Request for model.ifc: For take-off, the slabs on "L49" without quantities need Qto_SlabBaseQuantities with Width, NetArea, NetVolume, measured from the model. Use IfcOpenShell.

First a look at what the model holds.

```python
import ifcopenshell
import ifcopenshell.util.element
import ifcopenshell.util.unit

model = ifcopenshell.open("model.ifc")
print(model.schema)
for unit_type in ("LENGTHUNIT", "AREAUNIT", "VOLUMEUNIT"):
    print(unit_type, ifcopenshell.util.unit.calculate_unit_scale(model, unit_type))
storey = next(s for s in model.by_type("IfcBuildingStorey") if s.Name == "L49")
slabs = [e for e in ifcopenshell.util.element.get_decomposition(storey) if e.is_a("IfcSlab")]
for e in sorted(slabs, key=lambda e: e.id()):
    print(e.id(), e.is_a(), e.Name, list(ifcopenshell.util.element.get_psets(e, qtos_only=True)), sep=" | ")
```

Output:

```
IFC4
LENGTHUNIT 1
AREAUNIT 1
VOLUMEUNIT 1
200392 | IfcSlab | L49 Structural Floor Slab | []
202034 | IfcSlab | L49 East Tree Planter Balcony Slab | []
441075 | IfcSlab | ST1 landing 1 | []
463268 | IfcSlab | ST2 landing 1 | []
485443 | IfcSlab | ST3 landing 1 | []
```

```python
import ifcopenshell
import ifcopenshell.api.pset
import ifcopenshell.geom
import ifcopenshell.util.element
import ifcopenshell.util.shape
import ifcopenshell.util.unit

model = ifcopenshell.open("model.ifc")
unit_scale = ifcopenshell.util.unit.calculate_unit_scale(model)
area_scale = ifcopenshell.util.unit.calculate_unit_scale(model, "AREAUNIT")
volume_scale = ifcopenshell.util.unit.calculate_unit_scale(model, "VOLUMEUNIT")
settings = ifcopenshell.geom.settings()

storey = next(s for s in model.by_type("IfcBuildingStorey") if s.Name == "L49")
slabs = [e for e in ifcopenshell.util.element.get_decomposition(storey) if e.is_a("IfcSlab")]

for e in sorted(slabs, key=lambda e: e.id()):
    if ifcopenshell.util.element.get_psets(e, qtos_only=True, should_inherit=False):
        continue
    # Geometry comes back in metres, in the element's own axes.
    shape = ifcopenshell.geom.create_shape(settings, e)
    values = {
        "Width": ifcopenshell.util.shape.get_z(shape.geometry) / unit_scale,
        "NetArea": ifcopenshell.util.shape.get_footprint_area(shape.geometry) / area_scale,
        "NetVolume": ifcopenshell.util.shape.get_volume(shape.geometry) / volume_scale,
    }
    qto = ifcopenshell.api.pset.add_qto(model, product=e, name="Qto_SlabBaseQuantities")
    ifcopenshell.api.pset.edit_qto(model, qto=qto, properties=values)
    print(e.id(), {k: round(v, 3) for k, v in values.items()})

model.write("model_rev.ifc")
```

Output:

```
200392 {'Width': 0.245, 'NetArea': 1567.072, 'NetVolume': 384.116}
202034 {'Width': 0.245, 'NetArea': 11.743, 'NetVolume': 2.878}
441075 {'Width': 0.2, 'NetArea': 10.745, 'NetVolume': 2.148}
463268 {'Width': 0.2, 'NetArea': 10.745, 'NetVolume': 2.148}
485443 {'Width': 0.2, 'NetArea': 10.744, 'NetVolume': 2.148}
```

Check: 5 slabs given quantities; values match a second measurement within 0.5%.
